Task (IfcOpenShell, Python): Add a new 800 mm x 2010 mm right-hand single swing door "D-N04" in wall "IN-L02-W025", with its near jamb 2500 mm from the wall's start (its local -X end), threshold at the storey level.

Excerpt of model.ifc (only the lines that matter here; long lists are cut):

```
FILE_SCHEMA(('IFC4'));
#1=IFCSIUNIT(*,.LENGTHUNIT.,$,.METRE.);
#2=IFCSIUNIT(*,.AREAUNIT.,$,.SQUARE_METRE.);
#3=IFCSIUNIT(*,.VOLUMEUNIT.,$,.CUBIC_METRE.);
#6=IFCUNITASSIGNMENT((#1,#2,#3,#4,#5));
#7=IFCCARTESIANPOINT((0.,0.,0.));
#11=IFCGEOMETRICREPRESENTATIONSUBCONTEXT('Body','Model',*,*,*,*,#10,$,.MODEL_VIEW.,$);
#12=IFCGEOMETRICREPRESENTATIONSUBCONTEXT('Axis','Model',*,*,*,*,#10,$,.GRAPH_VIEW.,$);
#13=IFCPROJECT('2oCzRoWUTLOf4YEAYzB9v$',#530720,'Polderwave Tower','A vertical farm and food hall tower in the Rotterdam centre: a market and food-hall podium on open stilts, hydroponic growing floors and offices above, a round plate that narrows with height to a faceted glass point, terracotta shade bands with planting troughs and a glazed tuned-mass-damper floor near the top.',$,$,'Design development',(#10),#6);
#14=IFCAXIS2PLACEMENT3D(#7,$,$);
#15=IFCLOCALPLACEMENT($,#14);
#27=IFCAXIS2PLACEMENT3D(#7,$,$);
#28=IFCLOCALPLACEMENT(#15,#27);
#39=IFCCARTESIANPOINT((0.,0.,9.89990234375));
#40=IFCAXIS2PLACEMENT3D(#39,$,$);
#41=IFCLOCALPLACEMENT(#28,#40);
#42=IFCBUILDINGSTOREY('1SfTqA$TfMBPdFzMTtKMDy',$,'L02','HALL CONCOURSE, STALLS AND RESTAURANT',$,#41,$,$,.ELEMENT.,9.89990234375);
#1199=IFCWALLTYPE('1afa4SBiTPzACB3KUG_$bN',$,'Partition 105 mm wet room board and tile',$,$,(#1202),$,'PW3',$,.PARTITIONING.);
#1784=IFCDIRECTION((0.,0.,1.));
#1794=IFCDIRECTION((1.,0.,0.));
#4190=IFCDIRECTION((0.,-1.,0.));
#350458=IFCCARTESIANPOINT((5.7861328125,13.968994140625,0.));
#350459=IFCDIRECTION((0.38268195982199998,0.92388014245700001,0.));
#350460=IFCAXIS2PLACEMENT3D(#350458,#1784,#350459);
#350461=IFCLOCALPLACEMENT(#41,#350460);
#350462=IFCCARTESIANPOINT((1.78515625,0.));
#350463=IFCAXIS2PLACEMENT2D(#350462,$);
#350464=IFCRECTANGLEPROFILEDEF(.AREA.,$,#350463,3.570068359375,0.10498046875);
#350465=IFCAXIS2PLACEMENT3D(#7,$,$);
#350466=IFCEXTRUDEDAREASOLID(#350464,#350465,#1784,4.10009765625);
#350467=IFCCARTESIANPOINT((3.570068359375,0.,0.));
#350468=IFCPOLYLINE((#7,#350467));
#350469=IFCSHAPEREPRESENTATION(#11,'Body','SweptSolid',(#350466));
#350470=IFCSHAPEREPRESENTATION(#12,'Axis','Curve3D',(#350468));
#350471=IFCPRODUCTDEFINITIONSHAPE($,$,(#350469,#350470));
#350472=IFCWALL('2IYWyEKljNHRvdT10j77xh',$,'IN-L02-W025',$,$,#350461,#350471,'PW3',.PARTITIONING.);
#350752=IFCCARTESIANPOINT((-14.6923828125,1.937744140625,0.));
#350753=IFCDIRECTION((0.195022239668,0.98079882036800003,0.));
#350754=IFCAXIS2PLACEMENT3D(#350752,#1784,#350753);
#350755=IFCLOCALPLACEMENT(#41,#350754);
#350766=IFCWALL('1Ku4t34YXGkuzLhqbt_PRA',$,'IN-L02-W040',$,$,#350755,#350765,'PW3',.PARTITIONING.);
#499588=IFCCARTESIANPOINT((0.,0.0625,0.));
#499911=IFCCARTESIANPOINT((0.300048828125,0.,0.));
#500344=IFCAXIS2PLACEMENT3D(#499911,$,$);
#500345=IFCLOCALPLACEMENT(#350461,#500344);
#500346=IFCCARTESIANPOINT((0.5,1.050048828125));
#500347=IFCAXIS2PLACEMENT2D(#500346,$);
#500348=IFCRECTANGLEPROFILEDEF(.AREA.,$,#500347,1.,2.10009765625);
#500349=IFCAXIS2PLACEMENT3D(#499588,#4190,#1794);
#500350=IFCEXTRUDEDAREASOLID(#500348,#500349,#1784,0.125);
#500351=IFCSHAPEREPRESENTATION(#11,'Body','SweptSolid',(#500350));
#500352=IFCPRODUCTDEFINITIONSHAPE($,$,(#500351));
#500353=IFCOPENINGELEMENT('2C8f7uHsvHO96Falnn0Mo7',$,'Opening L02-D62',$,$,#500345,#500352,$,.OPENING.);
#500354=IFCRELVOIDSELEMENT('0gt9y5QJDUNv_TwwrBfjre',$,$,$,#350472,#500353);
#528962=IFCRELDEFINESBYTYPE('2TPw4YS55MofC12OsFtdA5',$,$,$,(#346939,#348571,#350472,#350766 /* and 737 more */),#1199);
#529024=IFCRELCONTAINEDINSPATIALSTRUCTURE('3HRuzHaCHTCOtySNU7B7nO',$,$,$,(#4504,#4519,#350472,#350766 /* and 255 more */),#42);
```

```python
import numpy as np
import ifcopenshell
import ifcopenshell.api.feature
import ifcopenshell.api.geometry
import ifcopenshell.api.root
import ifcopenshell.api.spatial
import ifcopenshell.geom
import ifcopenshell.util.element
import ifcopenshell.util.placement
import ifcopenshell.util.representation
import ifcopenshell.util.shape
import ifcopenshell.util.unit

model = ifcopenshell.open("model.ifc")
unit_scale = ifcopenshell.util.unit.calculate_unit_scale(model)
settings = ifcopenshell.geom.settings()


def volume(element):
    """Net volume in cubic metres, openings subtracted."""
    shape = ifcopenshell.geom.create_shape(settings, element)
    return ifcopenshell.util.shape.get_volume(shape.geometry)


wall = model.by_guid("2IYWyEKljNHRvdT10j77xh")
storey = ifcopenshell.util.element.get_container(wall, ifc_class="IfcBuildingStorey")
context = ifcopenshell.util.representation.get_context(model, "Model", "Body", "MODEL_VIEW")
before = volume(wall)

width, height, from_end, sill = 0.8, 2.01, 2.5, 0.0  # metres

# The wall runs along its own X axis, and the end named is its -X end.
wall_shape = ifcopenshell.geom.create_shape(settings, wall)
x, y, z = ifcopenshell.util.shape.get_vertices(wall_shape.geometry).T
start = x.min() + from_end
face, thickness = float(y.min()), float(y.max() - y.min())
wall_matrix = ifcopenshell.util.placement.get_local_placement(wall.ObjectPlacement)
level = ifcopenshell.util.placement.get_local_placement(storey.ObjectPlacement)[2, 3]


def in_wall(x, y):
    """Placement at x, y metres in the wall's axes, at sill height."""
    matrix = wall_matrix.copy()
    matrix[:, 3] = wall_matrix @ np.array([x / unit_scale, y / unit_scale, 0.0, 1.0])
    matrix[2, 3] = level + sill / unit_scale
    return matrix


# Opening: a box that overshoots both wall faces by 50 mm.
opening = ifcopenshell.api.root.create_entity(model, ifc_class="IfcOpeningElement", predefined_type="OPENING")
box = ifcopenshell.api.geometry.add_wall_representation(
    model, context=context, length=width, height=height, thickness=thickness + 0.1
)
ifcopenshell.api.geometry.assign_representation(model, product=opening, representation=box)
ifcopenshell.api.geometry.edit_object_placement(model, product=opening, matrix=in_wall(start, face - 0.05), is_si=False)
ifcopenshell.api.feature.add_feature(model, feature=opening, element=wall)

door = ifcopenshell.api.root.create_entity(model, ifc_class="IfcDoor", name="D-N04", predefined_type="DOOR")
door.OverallWidth, door.OverallHeight = width / unit_scale, height / unit_scale
door.OperationType = "SINGLE_SWING_RIGHT"
body = ifcopenshell.api.geometry.add_door_representation(
    model,
    context=context,
    overall_width=door.OverallWidth,
    overall_height=door.OverallHeight,
    operation_type="SINGLE_SWING_RIGHT",
    lining_properties={"LiningDepth": thickness / unit_scale, "ThresholdDepth": thickness / unit_scale},
)
ifcopenshell.api.geometry.assign_representation(model, product=door, representation=body)
ifcopenshell.api.spatial.assign_container(model, products=[door], relating_structure=storey)
ifcopenshell.api.feature.add_filling(model, opening=opening, element=door)

# The lining spans the wall, so the door starts at the wall face.
ifcopenshell.api.geometry.edit_object_placement(model, product=door, matrix=in_wall(start, face), is_si=False)

after = volume(wall)

print(f"wall volume {before:.3f} -> {after:.3f} m3")

model.write("model_v2.ifc")
```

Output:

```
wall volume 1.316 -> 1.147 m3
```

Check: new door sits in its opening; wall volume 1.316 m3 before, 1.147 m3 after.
